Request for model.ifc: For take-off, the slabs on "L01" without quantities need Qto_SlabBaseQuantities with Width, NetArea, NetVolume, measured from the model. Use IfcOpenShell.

First a look at what the model holds.

```python
import ifcopenshell
import ifcopenshell.util.element
import ifcopenshell.util.unit

model = ifcopenshell.open("model.ifc")
print(model.schema)
for unit_type in ("LENGTHUNIT", "AREAUNIT", "VOLUMEUNIT"):
    print(unit_type, ifcopenshell.util.unit.calculate_unit_scale(model, unit_type))
storey = next(s for s in model.by_type("IfcBuildingStorey") if s.Name == "L01")
slabs = [e for e in ifcopenshell.util.element.get_decomposition(storey) if e.is_a("IfcSlab")]
for e in sorted(slabs, key=lambda e: e.id()):
    print(e.id(), e.is_a(), e.Name, list(ifcopenshell.util.element.get_psets(e, qtos_only=True)), sep=" | ")
```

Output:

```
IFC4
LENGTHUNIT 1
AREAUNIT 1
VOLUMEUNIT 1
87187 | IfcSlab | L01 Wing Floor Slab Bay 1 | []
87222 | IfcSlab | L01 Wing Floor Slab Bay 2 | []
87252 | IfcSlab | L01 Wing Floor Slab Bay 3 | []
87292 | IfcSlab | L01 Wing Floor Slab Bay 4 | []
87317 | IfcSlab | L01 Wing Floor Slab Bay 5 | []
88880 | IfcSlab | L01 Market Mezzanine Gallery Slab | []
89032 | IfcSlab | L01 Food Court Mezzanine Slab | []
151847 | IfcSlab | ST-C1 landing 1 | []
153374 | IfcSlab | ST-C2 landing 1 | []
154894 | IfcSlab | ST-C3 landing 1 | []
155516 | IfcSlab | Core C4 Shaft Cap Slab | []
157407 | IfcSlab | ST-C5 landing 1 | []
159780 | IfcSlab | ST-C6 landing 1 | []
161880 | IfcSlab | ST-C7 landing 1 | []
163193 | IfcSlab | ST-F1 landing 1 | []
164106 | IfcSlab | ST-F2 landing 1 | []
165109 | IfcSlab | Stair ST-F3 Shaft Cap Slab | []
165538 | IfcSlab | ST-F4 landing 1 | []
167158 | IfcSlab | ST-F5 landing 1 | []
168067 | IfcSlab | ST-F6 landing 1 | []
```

```python
import ifcopenshell
import ifcopenshell.api.pset
import ifcopenshell.geom
import ifcopenshell.util.element
import ifcopenshell.util.shape
import ifcopenshell.util.unit

model = ifcopenshell.open("model.ifc")
unit_scale = ifcopenshell.util.unit.calculate_unit_scale(model)
area_scale = ifcopenshell.util.unit.calculate_unit_scale(model, "AREAUNIT")
volume_scale = ifcopenshell.util.unit.calculate_unit_scale(model, "VOLUMEUNIT")
settings = ifcopenshell.geom.settings()

storey = next(s for s in model.by_type("IfcBuildingStorey") if s.Name == "L01")
slabs = [e for e in ifcopenshell.util.element.get_decomposition(storey) if e.is_a("IfcSlab")]

for e in sorted(slabs, key=lambda e: e.id()):
    if ifcopenshell.util.element.get_psets(e, qtos_only=True, should_inherit=False):
        continue
    # Geometry comes back in metres, in the element's own axes.
    shape = ifcopenshell.geom.create_shape(settings, e)
    values = {
        "Width": ifcopenshell.util.shape.get_z(shape.geometry) / unit_scale,
        "NetArea": ifcopenshell.util.shape.get_footprint_area(shape.geometry) / area_scale,
        "NetVolume": ifcopenshell.util.shape.get_volume(shape.geometry) / volume_scale,
    }
    qto = ifcopenshell.api.pset.add_qto(model, product=e, name="Qto_SlabBaseQuantities")
    ifcopenshell.api.pset.edit_qto(model, qto=qto, properties=values)
    print(e.id(), {k: round(v, 3) for k, v in values.items()})

model.write("model_rev.ifc")
```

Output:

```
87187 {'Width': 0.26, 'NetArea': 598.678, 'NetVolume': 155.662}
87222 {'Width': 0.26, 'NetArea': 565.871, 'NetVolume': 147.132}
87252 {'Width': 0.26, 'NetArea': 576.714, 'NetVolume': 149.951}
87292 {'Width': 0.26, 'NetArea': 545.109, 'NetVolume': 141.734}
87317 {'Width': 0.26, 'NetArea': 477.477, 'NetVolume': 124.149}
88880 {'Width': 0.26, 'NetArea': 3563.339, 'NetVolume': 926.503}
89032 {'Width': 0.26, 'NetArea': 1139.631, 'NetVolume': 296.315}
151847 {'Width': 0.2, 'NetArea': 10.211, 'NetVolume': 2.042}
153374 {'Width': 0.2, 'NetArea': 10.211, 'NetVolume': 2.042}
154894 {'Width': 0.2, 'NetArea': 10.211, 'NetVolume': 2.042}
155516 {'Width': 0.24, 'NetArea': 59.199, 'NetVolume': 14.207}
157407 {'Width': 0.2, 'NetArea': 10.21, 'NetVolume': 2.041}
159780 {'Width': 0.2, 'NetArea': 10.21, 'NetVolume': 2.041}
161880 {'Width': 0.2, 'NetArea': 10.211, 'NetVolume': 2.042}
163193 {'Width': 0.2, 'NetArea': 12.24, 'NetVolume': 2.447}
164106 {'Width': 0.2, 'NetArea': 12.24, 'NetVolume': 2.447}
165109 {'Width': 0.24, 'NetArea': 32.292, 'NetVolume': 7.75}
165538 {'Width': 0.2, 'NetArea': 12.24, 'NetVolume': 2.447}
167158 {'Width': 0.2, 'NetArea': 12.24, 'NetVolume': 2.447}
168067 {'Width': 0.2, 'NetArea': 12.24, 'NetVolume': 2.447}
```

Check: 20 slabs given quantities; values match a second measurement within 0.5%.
